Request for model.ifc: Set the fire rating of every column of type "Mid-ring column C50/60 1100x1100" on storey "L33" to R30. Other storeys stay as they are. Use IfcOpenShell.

First a look at what the model holds.

```python
import ifcopenshell
import ifcopenshell.util.element

model = ifcopenshell.open("model.ifc")
print(model.schema)
storey = next(s for s in model.by_type("IfcBuildingStorey") if s.Name == "L33")
columns = [e for e in ifcopenshell.util.element.get_decomposition(storey) if e.is_a("IfcColumn")]
seen = {}
for e in columns:
    element_type = ifcopenshell.util.element.get_type(e)
    key = (element_type.Name if element_type != e and element_type else None, ifcopenshell.util.element.get_pset(e, "Pset_ColumnCommon", "FireRating"))
    seen[key] = seen.get(key, 0) + 1
for (name, value), count in sorted(seen.items(), key=str):
    print(count, "x", name, "|", value)
```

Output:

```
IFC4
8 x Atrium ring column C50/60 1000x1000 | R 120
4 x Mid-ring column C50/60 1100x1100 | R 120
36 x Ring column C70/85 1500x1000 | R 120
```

```python
import ifcopenshell
import ifcopenshell.api.pset
import ifcopenshell.util.element

model = ifcopenshell.open("model.ifc")

storey = next(s for s in model.by_type("IfcBuildingStorey") if s.Name == "L33")
columns = [e for e in ifcopenshell.util.element.get_decomposition(storey) if e.is_a("IfcColumn")]

count = 0
for e in columns:
    element_type = ifcopenshell.util.element.get_type(e)
    if element_type in (None, e) or element_type.Name != "Mid-ring column C50/60 1100x1100":
        continue
    found = ifcopenshell.util.element.get_pset(e, "Pset_ColumnCommon", should_inherit=False)
    if found:
        pset = model.by_id(found["id"])
        if len(ifcopenshell.util.element.get_elements_by_pset(pset)) > 1:
            pset = ifcopenshell.api.pset.unshare_pset(model, products=[e], pset=pset)[0]
    else:
        pset = ifcopenshell.api.pset.add_pset(model, product=e, name="Pset_ColumnCommon")
    ifcopenshell.api.pset.edit_pset(model, pset=pset, properties={"FireRating": "R30"})
    count += 1

print(count, "columns updated")

model.write("model_edited.ifc")
```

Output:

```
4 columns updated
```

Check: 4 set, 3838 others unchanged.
